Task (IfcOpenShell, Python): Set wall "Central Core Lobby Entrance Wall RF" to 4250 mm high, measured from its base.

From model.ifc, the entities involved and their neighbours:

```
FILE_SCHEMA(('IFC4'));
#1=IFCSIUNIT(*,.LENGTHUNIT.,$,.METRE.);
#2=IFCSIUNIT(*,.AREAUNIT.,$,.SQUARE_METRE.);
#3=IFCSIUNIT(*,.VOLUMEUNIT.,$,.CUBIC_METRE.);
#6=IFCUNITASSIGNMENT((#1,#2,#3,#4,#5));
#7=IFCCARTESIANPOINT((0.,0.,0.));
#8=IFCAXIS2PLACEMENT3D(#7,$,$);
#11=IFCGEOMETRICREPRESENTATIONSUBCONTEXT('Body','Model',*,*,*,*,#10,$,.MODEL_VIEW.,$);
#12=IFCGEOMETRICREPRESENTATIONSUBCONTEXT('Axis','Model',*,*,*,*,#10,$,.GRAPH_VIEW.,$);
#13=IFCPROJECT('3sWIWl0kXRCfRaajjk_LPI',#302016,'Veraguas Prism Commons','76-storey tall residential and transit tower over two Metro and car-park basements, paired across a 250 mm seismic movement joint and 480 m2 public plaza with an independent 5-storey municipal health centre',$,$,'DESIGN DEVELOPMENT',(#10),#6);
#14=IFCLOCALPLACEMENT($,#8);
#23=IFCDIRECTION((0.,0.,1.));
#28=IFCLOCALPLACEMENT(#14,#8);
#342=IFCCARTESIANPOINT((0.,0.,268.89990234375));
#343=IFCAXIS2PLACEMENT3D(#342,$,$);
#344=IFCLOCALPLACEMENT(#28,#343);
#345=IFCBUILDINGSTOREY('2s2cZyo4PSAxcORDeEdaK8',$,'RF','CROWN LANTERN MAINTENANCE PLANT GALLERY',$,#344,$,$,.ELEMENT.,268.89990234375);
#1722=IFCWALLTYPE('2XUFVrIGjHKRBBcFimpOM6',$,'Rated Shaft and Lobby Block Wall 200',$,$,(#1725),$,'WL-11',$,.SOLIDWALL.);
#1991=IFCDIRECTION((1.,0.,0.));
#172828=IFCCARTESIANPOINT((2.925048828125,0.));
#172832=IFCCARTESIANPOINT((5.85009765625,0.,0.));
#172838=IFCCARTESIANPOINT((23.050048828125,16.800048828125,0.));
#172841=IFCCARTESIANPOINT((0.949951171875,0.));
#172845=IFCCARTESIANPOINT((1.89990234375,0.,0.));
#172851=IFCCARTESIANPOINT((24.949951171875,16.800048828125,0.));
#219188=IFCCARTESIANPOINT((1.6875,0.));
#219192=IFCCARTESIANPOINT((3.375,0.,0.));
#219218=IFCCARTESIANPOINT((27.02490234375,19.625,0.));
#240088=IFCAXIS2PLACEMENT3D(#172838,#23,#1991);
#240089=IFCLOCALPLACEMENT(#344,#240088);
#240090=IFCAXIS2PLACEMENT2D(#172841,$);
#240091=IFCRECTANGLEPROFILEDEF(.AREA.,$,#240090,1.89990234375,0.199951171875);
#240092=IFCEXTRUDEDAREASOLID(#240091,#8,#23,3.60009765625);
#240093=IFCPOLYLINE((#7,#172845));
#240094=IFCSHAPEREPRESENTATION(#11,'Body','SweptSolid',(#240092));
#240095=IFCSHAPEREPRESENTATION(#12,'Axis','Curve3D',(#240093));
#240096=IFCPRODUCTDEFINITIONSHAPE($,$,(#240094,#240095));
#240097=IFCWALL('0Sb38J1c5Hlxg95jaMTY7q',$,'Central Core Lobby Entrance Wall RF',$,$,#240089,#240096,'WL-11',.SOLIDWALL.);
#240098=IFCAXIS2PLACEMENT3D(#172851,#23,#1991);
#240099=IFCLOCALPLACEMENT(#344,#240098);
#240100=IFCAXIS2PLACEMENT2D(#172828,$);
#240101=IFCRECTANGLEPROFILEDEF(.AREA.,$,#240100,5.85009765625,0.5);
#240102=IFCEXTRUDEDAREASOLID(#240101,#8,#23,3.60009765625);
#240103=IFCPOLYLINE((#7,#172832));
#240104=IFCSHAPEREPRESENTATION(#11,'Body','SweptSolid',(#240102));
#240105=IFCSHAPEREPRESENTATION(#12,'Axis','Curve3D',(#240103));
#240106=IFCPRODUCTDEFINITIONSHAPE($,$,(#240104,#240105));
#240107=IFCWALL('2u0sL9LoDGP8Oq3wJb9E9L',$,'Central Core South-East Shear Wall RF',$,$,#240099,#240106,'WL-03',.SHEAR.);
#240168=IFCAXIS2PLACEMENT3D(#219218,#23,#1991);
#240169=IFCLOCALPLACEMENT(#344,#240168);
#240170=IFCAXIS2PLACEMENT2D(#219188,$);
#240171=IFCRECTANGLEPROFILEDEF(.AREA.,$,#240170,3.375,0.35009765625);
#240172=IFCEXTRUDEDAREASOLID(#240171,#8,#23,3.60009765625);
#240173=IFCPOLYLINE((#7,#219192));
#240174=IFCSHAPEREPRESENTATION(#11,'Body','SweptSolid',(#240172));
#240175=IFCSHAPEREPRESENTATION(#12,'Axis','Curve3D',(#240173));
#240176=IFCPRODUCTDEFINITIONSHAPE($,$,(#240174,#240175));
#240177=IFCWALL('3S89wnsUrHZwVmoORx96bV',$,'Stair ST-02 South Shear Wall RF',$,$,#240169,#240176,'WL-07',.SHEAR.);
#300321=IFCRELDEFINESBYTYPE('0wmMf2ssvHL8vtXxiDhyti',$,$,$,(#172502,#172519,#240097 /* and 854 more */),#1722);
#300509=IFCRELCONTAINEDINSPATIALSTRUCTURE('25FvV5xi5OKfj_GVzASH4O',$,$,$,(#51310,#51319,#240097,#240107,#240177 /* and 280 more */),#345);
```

```python
import ifcopenshell
import ifcopenshell.geom
import ifcopenshell.util.representation
import ifcopenshell.util.shape

model = ifcopenshell.open("model.ifc")
settings = ifcopenshell.geom.settings()


def volume(element):
    """Net volume in cubic metres, openings subtracted."""
    shape = ifcopenshell.geom.create_shape(settings, element)
    return ifcopenshell.util.shape.get_volume(shape.geometry)


wall = model.by_guid("0Sb38J1c5Hlxg95jaMTY7q")
before = volume(wall)

body = ifcopenshell.util.representation.get_representation(wall, "Model", "Body")
solid = body.Items[0]
old_height = solid.Depth
solid.Depth = 4.25
after = volume(wall)

print(f"height {old_height:g} -> {solid.Depth:g}, volume {before:.3f} -> {after:.3f} m3")

model.write("model_rev.ifc")
```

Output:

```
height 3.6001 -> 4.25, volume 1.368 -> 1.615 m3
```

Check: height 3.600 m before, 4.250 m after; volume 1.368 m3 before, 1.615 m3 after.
